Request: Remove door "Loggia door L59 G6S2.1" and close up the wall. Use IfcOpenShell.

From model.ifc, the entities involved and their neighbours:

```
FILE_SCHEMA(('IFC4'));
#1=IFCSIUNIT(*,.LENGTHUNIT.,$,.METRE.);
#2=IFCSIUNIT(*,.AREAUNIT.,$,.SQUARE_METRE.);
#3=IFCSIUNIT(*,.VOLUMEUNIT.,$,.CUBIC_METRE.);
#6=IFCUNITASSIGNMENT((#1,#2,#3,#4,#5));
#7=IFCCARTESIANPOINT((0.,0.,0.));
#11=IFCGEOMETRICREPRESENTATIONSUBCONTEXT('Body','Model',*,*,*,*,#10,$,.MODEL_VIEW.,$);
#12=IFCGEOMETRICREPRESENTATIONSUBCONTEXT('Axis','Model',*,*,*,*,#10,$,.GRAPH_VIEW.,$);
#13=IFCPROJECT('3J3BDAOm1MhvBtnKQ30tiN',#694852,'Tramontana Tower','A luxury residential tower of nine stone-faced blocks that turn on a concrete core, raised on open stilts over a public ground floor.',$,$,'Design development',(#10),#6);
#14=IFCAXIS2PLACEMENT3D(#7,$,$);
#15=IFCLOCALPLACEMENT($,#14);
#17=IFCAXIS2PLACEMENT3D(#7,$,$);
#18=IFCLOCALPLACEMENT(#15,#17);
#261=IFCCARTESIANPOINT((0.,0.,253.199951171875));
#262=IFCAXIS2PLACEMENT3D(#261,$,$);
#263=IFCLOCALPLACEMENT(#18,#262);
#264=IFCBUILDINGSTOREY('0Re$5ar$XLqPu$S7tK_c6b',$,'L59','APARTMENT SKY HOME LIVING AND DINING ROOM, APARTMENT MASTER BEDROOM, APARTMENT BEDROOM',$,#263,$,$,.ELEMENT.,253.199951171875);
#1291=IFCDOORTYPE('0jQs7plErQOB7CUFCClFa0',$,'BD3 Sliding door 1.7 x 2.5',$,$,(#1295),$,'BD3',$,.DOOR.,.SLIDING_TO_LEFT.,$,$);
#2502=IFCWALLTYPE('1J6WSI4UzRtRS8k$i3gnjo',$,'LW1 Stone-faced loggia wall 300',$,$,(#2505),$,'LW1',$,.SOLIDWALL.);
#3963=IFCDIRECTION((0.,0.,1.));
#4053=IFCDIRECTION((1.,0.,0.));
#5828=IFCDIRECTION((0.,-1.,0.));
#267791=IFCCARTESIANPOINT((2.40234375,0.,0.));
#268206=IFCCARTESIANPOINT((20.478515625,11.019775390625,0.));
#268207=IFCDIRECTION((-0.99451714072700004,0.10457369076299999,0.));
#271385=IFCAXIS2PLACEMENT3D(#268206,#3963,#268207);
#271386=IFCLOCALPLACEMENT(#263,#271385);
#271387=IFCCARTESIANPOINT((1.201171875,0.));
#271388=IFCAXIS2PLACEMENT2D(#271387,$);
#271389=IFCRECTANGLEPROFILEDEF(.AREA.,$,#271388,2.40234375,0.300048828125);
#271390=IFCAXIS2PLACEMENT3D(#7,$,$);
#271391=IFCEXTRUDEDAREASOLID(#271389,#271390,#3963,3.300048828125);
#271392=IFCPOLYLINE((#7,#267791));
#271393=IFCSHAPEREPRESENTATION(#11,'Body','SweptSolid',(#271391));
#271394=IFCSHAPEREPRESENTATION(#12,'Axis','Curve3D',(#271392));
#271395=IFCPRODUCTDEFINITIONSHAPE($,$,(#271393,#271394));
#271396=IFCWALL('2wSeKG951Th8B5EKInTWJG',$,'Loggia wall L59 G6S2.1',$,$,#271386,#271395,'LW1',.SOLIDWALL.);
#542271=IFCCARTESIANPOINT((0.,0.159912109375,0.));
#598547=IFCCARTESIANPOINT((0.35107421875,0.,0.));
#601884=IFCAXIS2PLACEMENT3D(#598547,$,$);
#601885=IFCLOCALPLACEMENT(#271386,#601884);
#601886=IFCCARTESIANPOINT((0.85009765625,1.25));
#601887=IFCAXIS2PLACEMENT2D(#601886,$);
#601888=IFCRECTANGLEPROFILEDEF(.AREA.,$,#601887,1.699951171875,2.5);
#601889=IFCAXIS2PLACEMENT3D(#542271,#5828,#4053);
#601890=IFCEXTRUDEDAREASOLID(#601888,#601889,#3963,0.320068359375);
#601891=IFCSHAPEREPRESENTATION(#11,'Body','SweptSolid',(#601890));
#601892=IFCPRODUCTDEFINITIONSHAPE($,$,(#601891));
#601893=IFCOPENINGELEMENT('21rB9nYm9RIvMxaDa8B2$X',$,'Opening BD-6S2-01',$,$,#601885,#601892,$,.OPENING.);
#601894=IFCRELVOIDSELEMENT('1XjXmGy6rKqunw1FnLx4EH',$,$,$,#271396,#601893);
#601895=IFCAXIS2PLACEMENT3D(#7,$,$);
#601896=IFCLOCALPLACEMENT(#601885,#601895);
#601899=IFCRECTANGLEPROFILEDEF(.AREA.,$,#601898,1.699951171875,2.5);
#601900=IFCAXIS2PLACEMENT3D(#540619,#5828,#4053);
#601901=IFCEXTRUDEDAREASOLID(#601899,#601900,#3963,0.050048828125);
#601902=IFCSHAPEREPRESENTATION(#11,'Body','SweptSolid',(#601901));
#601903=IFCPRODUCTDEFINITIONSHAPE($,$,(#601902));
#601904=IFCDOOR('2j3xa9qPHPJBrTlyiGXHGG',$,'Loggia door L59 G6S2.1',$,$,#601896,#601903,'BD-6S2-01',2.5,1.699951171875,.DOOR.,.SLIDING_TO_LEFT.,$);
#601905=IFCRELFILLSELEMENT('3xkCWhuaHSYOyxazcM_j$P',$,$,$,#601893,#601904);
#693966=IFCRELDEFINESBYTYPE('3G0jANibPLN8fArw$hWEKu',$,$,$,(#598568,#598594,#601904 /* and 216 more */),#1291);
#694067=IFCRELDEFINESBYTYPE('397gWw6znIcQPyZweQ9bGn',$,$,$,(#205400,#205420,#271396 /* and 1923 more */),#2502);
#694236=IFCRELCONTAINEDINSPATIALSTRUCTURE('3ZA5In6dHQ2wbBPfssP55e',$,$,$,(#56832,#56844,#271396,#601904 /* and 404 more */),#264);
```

```python
import ifcopenshell
import ifcopenshell.api.feature
import ifcopenshell.api.root
import ifcopenshell.geom
import ifcopenshell.util.shape

model = ifcopenshell.open("model.ifc")
settings = ifcopenshell.geom.settings()


def volume(element):
    """Net volume in cubic metres, openings subtracted."""
    shape = ifcopenshell.geom.create_shape(settings, element)
    return ifcopenshell.util.shape.get_volume(shape.geometry)


door = model.by_id(601904)
opening = door.FillsVoids[0].RelatingOpeningElement
wall = opening.VoidsElements[0].RelatingBuildingElement
before = volume(wall)

ifcopenshell.api.root.remove_product(model, product=door)
ifcopenshell.api.feature.remove_feature(model, feature=opening)

after = volume(wall)

print(f"wall volume {before:.3f} -> {after:.3f} m3")

model.write("model_v2.ifc")
```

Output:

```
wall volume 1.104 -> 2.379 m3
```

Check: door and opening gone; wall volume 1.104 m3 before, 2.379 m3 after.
